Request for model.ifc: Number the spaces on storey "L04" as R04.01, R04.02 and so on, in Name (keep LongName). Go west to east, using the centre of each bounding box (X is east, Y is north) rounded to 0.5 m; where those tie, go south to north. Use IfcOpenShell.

First a look at what the model holds.

```python
import ifcopenshell
import ifcopenshell.util.element
import ifcopenshell.util.placement

model = ifcopenshell.open("model.ifc")
print(model.schema)
storey = next(s for s in model.by_type("IfcBuildingStorey") if s.Name == "L04")
spaces = [e for e in ifcopenshell.util.element.get_decomposition(storey) if e.is_a("IfcSpace")]
for e in sorted(spaces, key=lambda e: e.id()):
    origin = ifcopenshell.util.placement.get_local_placement(e.ObjectPlacement)[:3, 3]
    print(e.id(), e.Name, e.LongName, origin.round(2) + 0.0, sep=" | ")
```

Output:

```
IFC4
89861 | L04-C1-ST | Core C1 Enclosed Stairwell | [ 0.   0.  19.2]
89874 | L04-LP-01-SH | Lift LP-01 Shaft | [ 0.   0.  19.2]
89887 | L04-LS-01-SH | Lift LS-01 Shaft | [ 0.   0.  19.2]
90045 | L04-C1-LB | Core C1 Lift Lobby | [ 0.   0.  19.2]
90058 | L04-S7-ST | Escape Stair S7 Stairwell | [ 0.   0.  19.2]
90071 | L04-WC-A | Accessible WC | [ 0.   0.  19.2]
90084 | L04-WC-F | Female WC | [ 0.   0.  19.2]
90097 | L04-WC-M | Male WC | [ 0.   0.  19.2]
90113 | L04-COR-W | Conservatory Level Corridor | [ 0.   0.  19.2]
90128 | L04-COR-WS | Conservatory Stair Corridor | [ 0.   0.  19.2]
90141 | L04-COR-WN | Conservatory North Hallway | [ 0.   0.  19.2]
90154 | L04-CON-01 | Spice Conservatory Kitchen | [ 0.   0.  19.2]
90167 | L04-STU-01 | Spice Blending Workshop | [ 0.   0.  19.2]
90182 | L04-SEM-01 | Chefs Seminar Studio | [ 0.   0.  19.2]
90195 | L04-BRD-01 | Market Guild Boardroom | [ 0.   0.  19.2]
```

```python
import ifcopenshell
import ifcopenshell.geom
import ifcopenshell.util.element
import ifcopenshell.util.shape

model = ifcopenshell.open("model.ifc")
settings = ifcopenshell.geom.settings()
settings.set("use-world-coords", True)


def centre(element):
    shape = ifcopenshell.geom.create_shape(settings, element)
    return ifcopenshell.util.shape.get_bbox_centroid(shape.geometry)


storey = next(s for s in model.by_type("IfcBuildingStorey") if s.Name == "L04")
spaces = [e for e in ifcopenshell.util.element.get_decomposition(storey) if e.is_a("IfcSpace")]

# Insertion points can sit at a corner or the storey origin, so sort by the geometry (in metres).
centres = {e: centre(e) for e in spaces}
spaces.sort(key=lambda e: (round(centres[e][0] / 0.5), centres[e][1]))

for i, e in enumerate(spaces, start=1):
    number = f"R04.{i:02d}"
    e.Name = number
    print(e.id(), number)

model.write("model_v2.ifc")
```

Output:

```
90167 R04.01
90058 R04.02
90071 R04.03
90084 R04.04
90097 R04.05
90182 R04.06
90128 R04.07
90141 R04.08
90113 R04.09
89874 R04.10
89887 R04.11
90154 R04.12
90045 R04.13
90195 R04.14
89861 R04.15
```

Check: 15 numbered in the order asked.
